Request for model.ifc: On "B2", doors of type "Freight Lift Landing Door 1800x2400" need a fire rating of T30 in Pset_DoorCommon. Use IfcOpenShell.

First a look at what the model holds.

```python
import ifcopenshell
import ifcopenshell.util.element

model = ifcopenshell.open("model.ifc")
print(model.schema)
storey = next(s for s in model.by_type("IfcBuildingStorey") if s.Name == "B2")
doors = [e for e in ifcopenshell.util.element.get_decomposition(storey) if e.is_a("IfcDoor")]
seen = {}
for e in doors:
    element_type = ifcopenshell.util.element.get_type(e)
    key = (element_type.Name if element_type != e and element_type else None, ifcopenshell.util.element.get_pset(e, "Pset_DoorCommon", "FireRating"))
    seen[key] = seen.get(key, 0) + 1
for (name, value), count in sorted(seen.items(), key=str):
    print(count, "x", name, "|", value)
```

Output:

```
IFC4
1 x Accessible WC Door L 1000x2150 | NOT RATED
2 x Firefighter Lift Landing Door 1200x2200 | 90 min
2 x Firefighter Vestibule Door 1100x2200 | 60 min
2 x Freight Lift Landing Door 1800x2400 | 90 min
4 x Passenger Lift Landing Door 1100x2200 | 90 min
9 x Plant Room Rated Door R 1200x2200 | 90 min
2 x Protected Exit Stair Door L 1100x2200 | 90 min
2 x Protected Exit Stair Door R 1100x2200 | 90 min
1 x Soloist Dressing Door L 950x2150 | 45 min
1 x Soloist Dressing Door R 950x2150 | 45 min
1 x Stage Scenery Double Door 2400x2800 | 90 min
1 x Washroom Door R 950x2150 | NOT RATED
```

```python
import ifcopenshell
import ifcopenshell.api.pset
import ifcopenshell.util.element

model = ifcopenshell.open("model.ifc")

storey = next(s for s in model.by_type("IfcBuildingStorey") if s.Name == "B2")
doors = [e for e in ifcopenshell.util.element.get_decomposition(storey) if e.is_a("IfcDoor")]

count = 0
for e in doors:
    element_type = ifcopenshell.util.element.get_type(e)
    if element_type in (None, e) or element_type.Name != "Freight Lift Landing Door 1800x2400":
        continue
    # add_pset returns the element's existing set when there is one.
    pset = ifcopenshell.api.pset.add_pset(model, product=e, name="Pset_DoorCommon")
    ifcopenshell.api.pset.edit_pset(model, pset=pset, properties={"FireRating": "T30"})
    count += 1

print(count, "doors updated")

model.write("model_updated.ifc")
```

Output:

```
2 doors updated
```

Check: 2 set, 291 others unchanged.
